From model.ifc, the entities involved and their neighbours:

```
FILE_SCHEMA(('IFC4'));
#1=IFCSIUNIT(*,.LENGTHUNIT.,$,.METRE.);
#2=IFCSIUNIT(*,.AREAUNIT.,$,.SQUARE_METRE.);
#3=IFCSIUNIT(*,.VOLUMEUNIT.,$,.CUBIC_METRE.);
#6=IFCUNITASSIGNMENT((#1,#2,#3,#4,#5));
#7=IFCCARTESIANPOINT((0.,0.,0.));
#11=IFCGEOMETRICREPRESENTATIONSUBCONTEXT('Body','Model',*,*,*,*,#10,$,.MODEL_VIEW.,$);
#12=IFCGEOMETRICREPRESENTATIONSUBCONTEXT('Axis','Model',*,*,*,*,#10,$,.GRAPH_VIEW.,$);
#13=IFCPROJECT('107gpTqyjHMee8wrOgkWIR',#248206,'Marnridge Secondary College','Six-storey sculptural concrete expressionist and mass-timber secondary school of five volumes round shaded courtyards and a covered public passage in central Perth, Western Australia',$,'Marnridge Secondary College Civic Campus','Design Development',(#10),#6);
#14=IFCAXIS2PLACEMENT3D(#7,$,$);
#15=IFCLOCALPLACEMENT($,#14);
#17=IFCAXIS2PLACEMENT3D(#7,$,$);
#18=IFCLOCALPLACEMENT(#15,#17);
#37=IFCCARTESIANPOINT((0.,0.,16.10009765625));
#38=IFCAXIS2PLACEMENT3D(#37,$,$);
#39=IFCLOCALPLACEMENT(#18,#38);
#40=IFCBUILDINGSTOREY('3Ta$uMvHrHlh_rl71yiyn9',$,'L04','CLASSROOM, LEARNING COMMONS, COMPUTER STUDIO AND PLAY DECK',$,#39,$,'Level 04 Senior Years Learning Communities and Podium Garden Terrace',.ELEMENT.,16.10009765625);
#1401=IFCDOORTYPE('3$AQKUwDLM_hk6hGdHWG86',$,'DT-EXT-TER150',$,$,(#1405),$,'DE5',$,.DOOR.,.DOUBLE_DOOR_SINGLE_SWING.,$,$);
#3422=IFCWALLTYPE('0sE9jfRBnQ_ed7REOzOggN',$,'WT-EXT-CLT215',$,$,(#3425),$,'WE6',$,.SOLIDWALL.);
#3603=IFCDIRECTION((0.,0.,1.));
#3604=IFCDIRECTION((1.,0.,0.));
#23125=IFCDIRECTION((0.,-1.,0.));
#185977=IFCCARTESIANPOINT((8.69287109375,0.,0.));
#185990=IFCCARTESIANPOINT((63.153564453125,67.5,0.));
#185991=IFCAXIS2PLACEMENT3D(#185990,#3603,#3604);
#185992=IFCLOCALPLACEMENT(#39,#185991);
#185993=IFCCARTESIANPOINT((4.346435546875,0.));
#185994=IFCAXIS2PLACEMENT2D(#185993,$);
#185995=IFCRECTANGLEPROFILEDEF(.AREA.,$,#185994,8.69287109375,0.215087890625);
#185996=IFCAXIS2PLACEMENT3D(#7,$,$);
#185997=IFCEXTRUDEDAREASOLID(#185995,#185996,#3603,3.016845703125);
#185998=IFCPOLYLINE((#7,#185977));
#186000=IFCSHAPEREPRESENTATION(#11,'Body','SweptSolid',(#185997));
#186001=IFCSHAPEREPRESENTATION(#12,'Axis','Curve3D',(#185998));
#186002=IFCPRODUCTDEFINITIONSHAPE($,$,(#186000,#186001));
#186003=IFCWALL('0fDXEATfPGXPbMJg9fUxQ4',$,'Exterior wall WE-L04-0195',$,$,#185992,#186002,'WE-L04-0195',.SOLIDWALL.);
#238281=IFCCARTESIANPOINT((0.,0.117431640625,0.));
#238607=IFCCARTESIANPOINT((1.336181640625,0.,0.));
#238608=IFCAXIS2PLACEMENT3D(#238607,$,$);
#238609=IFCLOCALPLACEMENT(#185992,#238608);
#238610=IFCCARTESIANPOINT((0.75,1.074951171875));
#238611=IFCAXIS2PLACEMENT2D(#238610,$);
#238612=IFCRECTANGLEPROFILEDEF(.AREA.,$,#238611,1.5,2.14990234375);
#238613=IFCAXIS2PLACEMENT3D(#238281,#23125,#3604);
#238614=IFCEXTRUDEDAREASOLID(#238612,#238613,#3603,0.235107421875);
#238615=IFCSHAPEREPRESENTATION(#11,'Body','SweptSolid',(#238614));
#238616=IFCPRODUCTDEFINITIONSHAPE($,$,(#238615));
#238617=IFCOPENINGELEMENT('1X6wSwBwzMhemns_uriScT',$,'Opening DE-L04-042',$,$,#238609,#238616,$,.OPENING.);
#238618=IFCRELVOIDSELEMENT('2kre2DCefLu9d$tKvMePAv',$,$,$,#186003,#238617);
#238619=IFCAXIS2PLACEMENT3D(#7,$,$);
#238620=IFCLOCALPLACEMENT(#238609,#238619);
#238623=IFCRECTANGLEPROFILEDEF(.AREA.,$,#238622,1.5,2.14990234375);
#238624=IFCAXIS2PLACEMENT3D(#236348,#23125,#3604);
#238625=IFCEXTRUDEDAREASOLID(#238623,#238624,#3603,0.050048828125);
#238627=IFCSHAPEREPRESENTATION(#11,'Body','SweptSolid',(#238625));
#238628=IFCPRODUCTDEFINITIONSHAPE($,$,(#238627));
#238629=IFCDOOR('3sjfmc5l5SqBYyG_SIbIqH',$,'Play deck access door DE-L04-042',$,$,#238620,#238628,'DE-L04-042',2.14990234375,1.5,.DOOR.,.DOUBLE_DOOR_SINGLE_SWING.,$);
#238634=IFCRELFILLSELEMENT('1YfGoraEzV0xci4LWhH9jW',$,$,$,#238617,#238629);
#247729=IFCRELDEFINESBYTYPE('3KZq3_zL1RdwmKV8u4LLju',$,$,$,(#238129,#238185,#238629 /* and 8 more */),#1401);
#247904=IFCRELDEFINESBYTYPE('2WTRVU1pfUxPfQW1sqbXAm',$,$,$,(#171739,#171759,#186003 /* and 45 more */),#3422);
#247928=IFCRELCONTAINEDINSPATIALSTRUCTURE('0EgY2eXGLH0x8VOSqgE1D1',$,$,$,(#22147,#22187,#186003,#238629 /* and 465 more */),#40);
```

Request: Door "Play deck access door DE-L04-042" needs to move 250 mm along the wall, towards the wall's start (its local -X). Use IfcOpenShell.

```python
import ifcopenshell
import ifcopenshell.api.geometry
import ifcopenshell.util.placement
import ifcopenshell.util.unit

model = ifcopenshell.open("model.ifc")
unit_scale = ifcopenshell.util.unit.calculate_unit_scale(model)

door = model.by_guid("3sjfmc5l5SqBYyG_SIbIqH")
opening = door.FillsVoids[0].RelatingOpeningElement
wall = opening.VoidsElements[0].RelatingBuildingElement

wall_matrix = ifcopenshell.util.placement.get_local_placement(wall.ObjectPlacement)
shift = wall_matrix[:3, 0] * -0.25 / unit_scale
before = ifcopenshell.util.placement.get_local_placement(door.ObjectPlacement)[:3, 3].copy()

# The door is placed relative to its opening, so it follows when the opening moves.
matrix = ifcopenshell.util.placement.get_local_placement(opening.ObjectPlacement)
matrix[:3, 3] += shift
ifcopenshell.api.geometry.edit_object_placement(
    model, product=opening, matrix=matrix, is_si=False, should_transform_children=True
)

after = ifcopenshell.util.placement.get_local_placement(door.ObjectPlacement)[:3, 3]
print("door moved by", (after - before).round(3) + 0.0)

model.write("model_updated.ifc")
```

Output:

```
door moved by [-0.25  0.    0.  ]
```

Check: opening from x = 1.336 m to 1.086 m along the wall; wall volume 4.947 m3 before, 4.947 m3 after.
